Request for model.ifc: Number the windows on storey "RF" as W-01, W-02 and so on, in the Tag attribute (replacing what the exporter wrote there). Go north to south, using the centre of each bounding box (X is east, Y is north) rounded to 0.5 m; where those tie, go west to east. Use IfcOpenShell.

First a look at what the model holds.

```python
import ifcopenshell
import ifcopenshell.util.element
import ifcopenshell.util.placement

model = ifcopenshell.open("model.ifc")
print(model.schema)
storey = next(s for s in model.by_type("IfcBuildingStorey") if s.Name == "RF")
windows = [e for e in ifcopenshell.util.element.get_decomposition(storey) if e.is_a("IfcWindow")]
for e in sorted(windows, key=lambda e: e.id()):
    origin = ifcopenshell.util.placement.get_local_placement(e.ObjectPlacement)[:3, 3]
    print(e.id(), e.Tag, e.Name, origin.round(2) + 0.0, sep=" | ")
```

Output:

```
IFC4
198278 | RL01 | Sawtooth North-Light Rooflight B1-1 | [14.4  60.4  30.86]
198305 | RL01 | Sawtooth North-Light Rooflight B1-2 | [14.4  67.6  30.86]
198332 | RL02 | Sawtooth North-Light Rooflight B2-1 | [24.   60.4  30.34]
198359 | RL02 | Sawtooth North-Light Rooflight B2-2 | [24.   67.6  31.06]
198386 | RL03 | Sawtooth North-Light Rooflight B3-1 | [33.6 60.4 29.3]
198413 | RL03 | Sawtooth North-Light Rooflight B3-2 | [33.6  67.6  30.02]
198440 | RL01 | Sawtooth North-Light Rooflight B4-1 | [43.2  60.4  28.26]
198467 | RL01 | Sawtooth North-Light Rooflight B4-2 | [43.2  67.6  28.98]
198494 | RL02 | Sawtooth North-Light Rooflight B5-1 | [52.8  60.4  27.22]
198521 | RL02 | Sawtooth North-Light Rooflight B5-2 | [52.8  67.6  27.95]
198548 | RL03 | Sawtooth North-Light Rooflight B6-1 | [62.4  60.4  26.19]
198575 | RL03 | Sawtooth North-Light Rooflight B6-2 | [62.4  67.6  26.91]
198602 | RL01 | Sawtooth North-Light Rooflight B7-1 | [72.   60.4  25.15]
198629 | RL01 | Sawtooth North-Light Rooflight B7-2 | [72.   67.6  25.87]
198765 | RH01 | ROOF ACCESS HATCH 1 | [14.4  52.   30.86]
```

```python
import ifcopenshell
import ifcopenshell.geom
import ifcopenshell.util.element
import ifcopenshell.util.shape

model = ifcopenshell.open("model.ifc")
settings = ifcopenshell.geom.settings()
settings.set("use-world-coords", True)


def centre(element):
    shape = ifcopenshell.geom.create_shape(settings, element)
    return ifcopenshell.util.shape.get_bbox_centroid(shape.geometry)


storey = next(s for s in model.by_type("IfcBuildingStorey") if s.Name == "RF")
windows = [e for e in ifcopenshell.util.element.get_decomposition(storey) if e.is_a("IfcWindow")]

# Insertion points can sit at a corner or the storey origin, so sort by the geometry (in metres).
centres = {e: centre(e) for e in windows}
windows.sort(key=lambda e: (-round(centres[e][1] / 0.5), centres[e][0]))

for i, e in enumerate(windows, start=1):
    number = f"W-{i:02d}"
    e.Tag = number
    print(e.id(), number)

model.write("model_updated.ifc")
```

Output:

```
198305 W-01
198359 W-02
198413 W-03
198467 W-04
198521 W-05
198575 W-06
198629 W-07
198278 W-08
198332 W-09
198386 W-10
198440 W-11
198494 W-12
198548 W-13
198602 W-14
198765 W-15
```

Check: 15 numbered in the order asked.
